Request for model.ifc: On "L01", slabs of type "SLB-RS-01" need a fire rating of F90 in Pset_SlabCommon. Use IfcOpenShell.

First a look at what the model holds.

```python
import ifcopenshell
import ifcopenshell.util.element

model = ifcopenshell.open("model.ifc")
print(model.schema)
storey = next(s for s in model.by_type("IfcBuildingStorey") if s.Name == "L01")
slabs = [e for e in ifcopenshell.util.element.get_decomposition(storey) if e.is_a("IfcSlab")]
seen = {}
for e in slabs:
    element_type = ifcopenshell.util.element.get_type(e)
    key = (element_type.Name if element_type != e and element_type else None, ifcopenshell.util.element.get_pset(e, "Pset_SlabCommon", "FireRating"))
    seen[key] = seen.get(key, 0) + 1
for (name, value), count in sorted(seen.items(), key=str):
    print(count, "x", name, "|", value)
```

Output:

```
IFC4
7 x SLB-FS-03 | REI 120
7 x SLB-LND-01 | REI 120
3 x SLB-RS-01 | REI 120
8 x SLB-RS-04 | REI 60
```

```python
import ifcopenshell
import ifcopenshell.api.pset
import ifcopenshell.util.element

model = ifcopenshell.open("model.ifc")

storey = next(s for s in model.by_type("IfcBuildingStorey") if s.Name == "L01")
slabs = [e for e in ifcopenshell.util.element.get_decomposition(storey) if e.is_a("IfcSlab")]

count = 0
for e in slabs:
    element_type = ifcopenshell.util.element.get_type(e)
    if element_type in (None, e) or element_type.Name != "SLB-RS-01":
        continue
    # add_pset returns the element's existing set when there is one.
    pset = ifcopenshell.api.pset.add_pset(model, product=e, name="Pset_SlabCommon")
    ifcopenshell.api.pset.edit_pset(model, pset=pset, properties={"FireRating": "F90"})
    count += 1

print(count, "slabs updated")

model.write("model_updated.ifc")
```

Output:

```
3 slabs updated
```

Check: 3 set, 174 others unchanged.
